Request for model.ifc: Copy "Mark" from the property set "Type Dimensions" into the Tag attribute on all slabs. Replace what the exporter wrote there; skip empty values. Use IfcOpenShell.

First a look at what the model holds.

```python
import ifcopenshell
import ifcopenshell.util.element

model = ifcopenshell.open("model.ifc")
print(model.schema)
slabs = model.by_type("IfcSlab")
print(len(slabs), "slabs")
for e in slabs[:8]:
    source = ifcopenshell.util.element.get_pset(e, "Type Dimensions", "Mark")
    target = e.Tag
    print(e.id(), repr(source), repr(target), sep=" | ")
```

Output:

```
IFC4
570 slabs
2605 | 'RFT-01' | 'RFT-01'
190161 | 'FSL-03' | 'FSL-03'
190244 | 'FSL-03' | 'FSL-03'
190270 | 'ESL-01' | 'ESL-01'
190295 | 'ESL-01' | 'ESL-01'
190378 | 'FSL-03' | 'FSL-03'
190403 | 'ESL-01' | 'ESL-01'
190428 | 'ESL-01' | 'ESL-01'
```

```python
import ifcopenshell
import ifcopenshell.util.element

model = ifcopenshell.open("model.ifc")

count = 0
for e in model.by_type("IfcSlab"):
    value = ifcopenshell.util.element.get_pset(e, "Type Dimensions", "Mark")
    current = e.Tag
    if not value or not value.strip() or current == value:
        continue
    e.Tag = value
    count += 1

print(count, "slabs updated")

model.write("model-out.ifc")
```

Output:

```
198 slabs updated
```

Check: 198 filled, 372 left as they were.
